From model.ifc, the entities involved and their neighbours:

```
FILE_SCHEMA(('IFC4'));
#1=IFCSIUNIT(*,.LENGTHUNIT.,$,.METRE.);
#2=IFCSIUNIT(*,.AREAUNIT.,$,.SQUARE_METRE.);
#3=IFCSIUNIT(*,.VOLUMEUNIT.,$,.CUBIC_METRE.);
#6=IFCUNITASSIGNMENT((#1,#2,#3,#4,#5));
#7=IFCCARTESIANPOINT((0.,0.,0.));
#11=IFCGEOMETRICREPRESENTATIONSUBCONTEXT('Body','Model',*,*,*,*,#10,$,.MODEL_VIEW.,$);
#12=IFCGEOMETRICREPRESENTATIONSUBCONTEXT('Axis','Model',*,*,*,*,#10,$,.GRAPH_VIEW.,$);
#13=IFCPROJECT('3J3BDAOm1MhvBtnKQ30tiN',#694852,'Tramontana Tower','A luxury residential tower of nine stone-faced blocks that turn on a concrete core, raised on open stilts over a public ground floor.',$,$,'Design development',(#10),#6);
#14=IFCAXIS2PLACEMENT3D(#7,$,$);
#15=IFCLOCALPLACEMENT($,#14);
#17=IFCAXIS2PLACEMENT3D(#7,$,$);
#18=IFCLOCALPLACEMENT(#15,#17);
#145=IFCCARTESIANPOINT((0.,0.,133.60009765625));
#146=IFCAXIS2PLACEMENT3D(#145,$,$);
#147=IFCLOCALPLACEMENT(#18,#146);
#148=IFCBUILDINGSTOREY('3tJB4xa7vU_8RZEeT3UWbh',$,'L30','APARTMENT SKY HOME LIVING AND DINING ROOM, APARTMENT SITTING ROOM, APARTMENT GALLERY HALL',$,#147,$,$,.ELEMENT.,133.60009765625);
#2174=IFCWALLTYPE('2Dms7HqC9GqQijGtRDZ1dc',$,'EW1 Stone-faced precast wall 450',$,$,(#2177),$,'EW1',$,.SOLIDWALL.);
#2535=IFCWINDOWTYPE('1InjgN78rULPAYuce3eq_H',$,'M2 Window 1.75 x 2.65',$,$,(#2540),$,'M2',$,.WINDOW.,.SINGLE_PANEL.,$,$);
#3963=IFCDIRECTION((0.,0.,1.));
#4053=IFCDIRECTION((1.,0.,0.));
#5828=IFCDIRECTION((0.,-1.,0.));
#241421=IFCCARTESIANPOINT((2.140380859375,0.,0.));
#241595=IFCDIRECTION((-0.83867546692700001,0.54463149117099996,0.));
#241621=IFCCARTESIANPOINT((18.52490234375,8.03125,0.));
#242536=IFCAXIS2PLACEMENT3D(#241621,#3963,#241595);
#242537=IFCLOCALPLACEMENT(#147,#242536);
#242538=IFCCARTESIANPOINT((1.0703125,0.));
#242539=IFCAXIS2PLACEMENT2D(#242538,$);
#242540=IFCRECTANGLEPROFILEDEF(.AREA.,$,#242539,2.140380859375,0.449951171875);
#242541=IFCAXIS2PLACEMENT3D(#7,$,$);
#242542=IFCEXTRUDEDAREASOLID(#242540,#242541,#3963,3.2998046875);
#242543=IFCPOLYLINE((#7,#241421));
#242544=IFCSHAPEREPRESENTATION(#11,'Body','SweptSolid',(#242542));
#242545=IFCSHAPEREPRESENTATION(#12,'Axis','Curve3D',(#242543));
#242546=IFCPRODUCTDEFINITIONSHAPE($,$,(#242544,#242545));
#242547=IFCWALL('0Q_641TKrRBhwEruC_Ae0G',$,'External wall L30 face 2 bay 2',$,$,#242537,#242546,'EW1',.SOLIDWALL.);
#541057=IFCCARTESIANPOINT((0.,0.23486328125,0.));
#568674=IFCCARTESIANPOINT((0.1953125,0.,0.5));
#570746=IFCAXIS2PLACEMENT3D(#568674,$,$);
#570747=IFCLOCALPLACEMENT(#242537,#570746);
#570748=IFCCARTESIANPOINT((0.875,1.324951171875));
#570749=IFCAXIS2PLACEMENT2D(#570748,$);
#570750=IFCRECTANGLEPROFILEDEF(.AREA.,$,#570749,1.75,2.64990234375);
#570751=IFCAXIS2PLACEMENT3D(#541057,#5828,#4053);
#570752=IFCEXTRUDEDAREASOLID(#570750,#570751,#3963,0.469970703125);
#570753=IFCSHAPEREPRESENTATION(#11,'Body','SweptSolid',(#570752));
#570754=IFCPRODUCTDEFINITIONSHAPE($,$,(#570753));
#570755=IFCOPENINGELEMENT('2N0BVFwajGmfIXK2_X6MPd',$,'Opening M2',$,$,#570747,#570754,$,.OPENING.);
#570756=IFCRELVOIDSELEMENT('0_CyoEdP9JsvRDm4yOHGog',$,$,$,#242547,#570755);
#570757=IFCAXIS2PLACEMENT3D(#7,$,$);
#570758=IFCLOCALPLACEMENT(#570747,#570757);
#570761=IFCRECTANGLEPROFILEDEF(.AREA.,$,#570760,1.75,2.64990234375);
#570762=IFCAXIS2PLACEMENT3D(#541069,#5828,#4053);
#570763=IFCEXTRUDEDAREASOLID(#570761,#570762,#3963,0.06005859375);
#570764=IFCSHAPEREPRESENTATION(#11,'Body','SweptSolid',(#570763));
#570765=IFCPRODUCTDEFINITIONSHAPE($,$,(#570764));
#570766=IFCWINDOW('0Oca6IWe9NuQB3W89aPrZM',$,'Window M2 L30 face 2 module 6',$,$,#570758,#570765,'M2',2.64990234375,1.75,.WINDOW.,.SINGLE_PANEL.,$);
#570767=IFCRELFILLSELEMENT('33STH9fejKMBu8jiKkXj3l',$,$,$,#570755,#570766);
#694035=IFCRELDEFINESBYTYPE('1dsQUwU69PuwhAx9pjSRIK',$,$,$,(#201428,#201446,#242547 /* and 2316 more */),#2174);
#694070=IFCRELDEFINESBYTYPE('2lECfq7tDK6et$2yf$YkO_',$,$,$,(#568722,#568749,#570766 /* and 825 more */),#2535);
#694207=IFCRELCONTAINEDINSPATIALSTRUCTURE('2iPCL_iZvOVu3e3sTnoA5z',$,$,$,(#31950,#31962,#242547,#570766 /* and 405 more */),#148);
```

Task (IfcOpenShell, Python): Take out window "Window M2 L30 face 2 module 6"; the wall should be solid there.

```python
import ifcopenshell
import ifcopenshell.api.feature
import ifcopenshell.api.root
import ifcopenshell.geom
import ifcopenshell.util.shape

model = ifcopenshell.open("model.ifc")
settings = ifcopenshell.geom.settings()


def volume(element):
    """Net volume in cubic metres, openings subtracted."""
    shape = ifcopenshell.geom.create_shape(settings, element)
    return ifcopenshell.util.shape.get_volume(shape.geometry)


window = model.by_guid("0Oca6IWe9NuQB3W89aPrZM")
opening = window.FillsVoids[0].RelatingOpeningElement
wall = opening.VoidsElements[0].RelatingBuildingElement
before = volume(wall)

ifcopenshell.api.root.remove_product(model, product=window)
ifcopenshell.api.feature.remove_feature(model, feature=opening)

after = volume(wall)

print(f"wall volume {before:.3f} -> {after:.3f} m3")

model.write("model_edited.ifc")
```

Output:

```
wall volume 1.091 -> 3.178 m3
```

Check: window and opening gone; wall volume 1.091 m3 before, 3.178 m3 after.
